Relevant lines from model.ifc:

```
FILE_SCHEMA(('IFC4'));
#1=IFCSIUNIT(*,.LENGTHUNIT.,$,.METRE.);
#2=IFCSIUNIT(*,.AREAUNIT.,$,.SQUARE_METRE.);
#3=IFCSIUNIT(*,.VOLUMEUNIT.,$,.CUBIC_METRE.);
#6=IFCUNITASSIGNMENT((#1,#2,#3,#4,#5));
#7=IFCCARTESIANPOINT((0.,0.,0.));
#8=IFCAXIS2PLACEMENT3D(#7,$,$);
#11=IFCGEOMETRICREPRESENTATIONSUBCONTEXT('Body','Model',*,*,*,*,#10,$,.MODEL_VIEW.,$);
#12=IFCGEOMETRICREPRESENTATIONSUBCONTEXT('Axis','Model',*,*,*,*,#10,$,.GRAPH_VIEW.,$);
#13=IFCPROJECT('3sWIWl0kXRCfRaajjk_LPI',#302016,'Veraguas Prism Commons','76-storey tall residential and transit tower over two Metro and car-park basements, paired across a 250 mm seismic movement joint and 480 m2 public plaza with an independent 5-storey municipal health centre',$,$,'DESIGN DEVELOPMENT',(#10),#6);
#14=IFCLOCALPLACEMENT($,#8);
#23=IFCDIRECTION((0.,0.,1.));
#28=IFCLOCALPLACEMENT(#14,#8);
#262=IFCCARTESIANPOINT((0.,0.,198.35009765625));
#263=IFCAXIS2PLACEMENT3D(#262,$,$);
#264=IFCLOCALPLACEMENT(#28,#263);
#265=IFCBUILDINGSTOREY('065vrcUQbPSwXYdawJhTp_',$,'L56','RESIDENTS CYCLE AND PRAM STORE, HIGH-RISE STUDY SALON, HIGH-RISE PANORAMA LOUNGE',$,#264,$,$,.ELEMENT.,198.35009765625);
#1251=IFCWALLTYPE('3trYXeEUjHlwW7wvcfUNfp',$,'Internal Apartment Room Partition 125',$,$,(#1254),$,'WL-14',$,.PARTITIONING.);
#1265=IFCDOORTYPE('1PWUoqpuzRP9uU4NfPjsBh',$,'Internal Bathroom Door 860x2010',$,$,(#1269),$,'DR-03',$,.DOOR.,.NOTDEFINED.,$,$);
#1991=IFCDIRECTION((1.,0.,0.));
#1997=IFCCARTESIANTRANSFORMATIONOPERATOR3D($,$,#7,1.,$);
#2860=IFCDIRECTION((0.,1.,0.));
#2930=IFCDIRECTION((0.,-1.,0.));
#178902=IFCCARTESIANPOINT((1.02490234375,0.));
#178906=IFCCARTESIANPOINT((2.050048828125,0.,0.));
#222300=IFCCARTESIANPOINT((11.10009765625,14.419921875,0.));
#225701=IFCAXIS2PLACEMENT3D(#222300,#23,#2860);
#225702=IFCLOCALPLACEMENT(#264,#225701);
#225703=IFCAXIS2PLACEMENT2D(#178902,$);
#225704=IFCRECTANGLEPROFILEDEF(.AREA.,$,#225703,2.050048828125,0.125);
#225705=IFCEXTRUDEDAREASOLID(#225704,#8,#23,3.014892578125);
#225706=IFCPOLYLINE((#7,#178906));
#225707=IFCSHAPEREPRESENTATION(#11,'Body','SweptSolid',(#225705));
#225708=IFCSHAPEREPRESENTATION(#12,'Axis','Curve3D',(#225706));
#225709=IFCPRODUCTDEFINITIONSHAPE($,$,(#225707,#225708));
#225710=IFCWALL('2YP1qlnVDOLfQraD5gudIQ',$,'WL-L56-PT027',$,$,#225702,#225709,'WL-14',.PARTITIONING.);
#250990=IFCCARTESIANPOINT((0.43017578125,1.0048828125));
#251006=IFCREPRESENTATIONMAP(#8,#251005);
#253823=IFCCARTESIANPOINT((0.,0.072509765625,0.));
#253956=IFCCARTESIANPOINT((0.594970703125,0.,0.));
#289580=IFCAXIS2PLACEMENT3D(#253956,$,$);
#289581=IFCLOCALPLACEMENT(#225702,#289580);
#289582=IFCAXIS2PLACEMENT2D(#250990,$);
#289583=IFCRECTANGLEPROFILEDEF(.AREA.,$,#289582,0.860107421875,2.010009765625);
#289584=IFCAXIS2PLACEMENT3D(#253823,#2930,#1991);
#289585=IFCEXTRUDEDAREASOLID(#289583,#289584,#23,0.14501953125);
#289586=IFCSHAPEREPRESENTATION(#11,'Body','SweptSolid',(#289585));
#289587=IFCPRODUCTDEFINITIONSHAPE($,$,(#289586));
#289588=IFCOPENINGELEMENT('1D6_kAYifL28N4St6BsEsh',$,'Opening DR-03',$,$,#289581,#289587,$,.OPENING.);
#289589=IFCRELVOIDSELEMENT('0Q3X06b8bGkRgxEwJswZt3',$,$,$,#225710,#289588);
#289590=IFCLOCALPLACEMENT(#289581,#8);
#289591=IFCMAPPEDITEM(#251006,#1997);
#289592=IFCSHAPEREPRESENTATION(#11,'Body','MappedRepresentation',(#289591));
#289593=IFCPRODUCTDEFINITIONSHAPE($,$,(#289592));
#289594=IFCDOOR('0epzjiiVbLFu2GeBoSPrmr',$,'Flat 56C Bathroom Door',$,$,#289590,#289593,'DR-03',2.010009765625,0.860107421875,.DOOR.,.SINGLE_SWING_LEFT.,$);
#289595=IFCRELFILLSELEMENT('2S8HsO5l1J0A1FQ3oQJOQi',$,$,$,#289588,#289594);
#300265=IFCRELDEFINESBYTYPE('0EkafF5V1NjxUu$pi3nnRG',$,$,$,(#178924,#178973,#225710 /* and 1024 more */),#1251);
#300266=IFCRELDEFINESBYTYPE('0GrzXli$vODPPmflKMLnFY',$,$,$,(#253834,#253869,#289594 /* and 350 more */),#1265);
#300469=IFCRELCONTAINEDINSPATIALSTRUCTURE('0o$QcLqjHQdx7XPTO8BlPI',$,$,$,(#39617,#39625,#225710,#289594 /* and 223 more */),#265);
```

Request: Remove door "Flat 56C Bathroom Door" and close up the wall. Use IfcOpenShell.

```python
import ifcopenshell
import ifcopenshell.api.feature
import ifcopenshell.api.root
import ifcopenshell.geom
import ifcopenshell.util.shape

model = ifcopenshell.open("model.ifc")
settings = ifcopenshell.geom.settings()


def volume(element):
    """Net volume in cubic metres, openings subtracted."""
    shape = ifcopenshell.geom.create_shape(settings, element)
    return ifcopenshell.util.shape.get_volume(shape.geometry)


door = model.by_guid("0epzjiiVbLFu2GeBoSPrmr")
opening = door.FillsVoids[0].RelatingOpeningElement
wall = opening.VoidsElements[0].RelatingBuildingElement
before = volume(wall)

ifcopenshell.api.root.remove_product(model, product=door)
ifcopenshell.api.feature.remove_feature(model, feature=opening)

after = volume(wall)

print(f"wall volume {before:.3f} -> {after:.3f} m3")

model.write("model_updated.ifc")
```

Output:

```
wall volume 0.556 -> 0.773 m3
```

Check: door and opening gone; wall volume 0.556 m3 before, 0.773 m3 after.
